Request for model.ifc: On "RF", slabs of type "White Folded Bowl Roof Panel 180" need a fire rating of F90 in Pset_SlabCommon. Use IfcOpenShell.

First a look at what the model holds.

```python
import ifcopenshell
import ifcopenshell.util.element

model = ifcopenshell.open("model.ifc")
print(model.schema)
storey = next(s for s in model.by_type("IfcBuildingStorey") if s.Name == "RF")
slabs = [e for e in ifcopenshell.util.element.get_decomposition(storey) if e.is_a("IfcSlab")]
seen = {}
for e in slabs:
    element_type = ifcopenshell.util.element.get_type(e)
    key = (element_type.Name if element_type != e and element_type else None, ifcopenshell.util.element.get_pset(e, "Pset_SlabCommon", "FireRating"))
    seen[key] = seen.get(key, 0) + 1
for (name, value), count in sorted(seen.items(), key=str):
    print(count, "x", name, "|", value)
```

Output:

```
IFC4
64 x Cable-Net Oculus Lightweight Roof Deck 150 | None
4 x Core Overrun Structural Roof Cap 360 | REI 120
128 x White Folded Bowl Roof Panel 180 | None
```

```python
import ifcopenshell
import ifcopenshell.api.pset
import ifcopenshell.util.element

model = ifcopenshell.open("model.ifc")

storey = next(s for s in model.by_type("IfcBuildingStorey") if s.Name == "RF")
slabs = [e for e in ifcopenshell.util.element.get_decomposition(storey) if e.is_a("IfcSlab")]

count = 0
for e in slabs:
    element_type = ifcopenshell.util.element.get_type(e)
    if element_type in (None, e) or element_type.Name != "White Folded Bowl Roof Panel 180":
        continue
    # add_pset returns the element's existing set when there is one.
    pset = ifcopenshell.api.pset.add_pset(model, product=e, name="Pset_SlabCommon")
    ifcopenshell.api.pset.edit_pset(model, pset=pset, properties={"FireRating": "F90"})
    count += 1

print(count, "slabs updated")

model.write("model_rev.ifc")
```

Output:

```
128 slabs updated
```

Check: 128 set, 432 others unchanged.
